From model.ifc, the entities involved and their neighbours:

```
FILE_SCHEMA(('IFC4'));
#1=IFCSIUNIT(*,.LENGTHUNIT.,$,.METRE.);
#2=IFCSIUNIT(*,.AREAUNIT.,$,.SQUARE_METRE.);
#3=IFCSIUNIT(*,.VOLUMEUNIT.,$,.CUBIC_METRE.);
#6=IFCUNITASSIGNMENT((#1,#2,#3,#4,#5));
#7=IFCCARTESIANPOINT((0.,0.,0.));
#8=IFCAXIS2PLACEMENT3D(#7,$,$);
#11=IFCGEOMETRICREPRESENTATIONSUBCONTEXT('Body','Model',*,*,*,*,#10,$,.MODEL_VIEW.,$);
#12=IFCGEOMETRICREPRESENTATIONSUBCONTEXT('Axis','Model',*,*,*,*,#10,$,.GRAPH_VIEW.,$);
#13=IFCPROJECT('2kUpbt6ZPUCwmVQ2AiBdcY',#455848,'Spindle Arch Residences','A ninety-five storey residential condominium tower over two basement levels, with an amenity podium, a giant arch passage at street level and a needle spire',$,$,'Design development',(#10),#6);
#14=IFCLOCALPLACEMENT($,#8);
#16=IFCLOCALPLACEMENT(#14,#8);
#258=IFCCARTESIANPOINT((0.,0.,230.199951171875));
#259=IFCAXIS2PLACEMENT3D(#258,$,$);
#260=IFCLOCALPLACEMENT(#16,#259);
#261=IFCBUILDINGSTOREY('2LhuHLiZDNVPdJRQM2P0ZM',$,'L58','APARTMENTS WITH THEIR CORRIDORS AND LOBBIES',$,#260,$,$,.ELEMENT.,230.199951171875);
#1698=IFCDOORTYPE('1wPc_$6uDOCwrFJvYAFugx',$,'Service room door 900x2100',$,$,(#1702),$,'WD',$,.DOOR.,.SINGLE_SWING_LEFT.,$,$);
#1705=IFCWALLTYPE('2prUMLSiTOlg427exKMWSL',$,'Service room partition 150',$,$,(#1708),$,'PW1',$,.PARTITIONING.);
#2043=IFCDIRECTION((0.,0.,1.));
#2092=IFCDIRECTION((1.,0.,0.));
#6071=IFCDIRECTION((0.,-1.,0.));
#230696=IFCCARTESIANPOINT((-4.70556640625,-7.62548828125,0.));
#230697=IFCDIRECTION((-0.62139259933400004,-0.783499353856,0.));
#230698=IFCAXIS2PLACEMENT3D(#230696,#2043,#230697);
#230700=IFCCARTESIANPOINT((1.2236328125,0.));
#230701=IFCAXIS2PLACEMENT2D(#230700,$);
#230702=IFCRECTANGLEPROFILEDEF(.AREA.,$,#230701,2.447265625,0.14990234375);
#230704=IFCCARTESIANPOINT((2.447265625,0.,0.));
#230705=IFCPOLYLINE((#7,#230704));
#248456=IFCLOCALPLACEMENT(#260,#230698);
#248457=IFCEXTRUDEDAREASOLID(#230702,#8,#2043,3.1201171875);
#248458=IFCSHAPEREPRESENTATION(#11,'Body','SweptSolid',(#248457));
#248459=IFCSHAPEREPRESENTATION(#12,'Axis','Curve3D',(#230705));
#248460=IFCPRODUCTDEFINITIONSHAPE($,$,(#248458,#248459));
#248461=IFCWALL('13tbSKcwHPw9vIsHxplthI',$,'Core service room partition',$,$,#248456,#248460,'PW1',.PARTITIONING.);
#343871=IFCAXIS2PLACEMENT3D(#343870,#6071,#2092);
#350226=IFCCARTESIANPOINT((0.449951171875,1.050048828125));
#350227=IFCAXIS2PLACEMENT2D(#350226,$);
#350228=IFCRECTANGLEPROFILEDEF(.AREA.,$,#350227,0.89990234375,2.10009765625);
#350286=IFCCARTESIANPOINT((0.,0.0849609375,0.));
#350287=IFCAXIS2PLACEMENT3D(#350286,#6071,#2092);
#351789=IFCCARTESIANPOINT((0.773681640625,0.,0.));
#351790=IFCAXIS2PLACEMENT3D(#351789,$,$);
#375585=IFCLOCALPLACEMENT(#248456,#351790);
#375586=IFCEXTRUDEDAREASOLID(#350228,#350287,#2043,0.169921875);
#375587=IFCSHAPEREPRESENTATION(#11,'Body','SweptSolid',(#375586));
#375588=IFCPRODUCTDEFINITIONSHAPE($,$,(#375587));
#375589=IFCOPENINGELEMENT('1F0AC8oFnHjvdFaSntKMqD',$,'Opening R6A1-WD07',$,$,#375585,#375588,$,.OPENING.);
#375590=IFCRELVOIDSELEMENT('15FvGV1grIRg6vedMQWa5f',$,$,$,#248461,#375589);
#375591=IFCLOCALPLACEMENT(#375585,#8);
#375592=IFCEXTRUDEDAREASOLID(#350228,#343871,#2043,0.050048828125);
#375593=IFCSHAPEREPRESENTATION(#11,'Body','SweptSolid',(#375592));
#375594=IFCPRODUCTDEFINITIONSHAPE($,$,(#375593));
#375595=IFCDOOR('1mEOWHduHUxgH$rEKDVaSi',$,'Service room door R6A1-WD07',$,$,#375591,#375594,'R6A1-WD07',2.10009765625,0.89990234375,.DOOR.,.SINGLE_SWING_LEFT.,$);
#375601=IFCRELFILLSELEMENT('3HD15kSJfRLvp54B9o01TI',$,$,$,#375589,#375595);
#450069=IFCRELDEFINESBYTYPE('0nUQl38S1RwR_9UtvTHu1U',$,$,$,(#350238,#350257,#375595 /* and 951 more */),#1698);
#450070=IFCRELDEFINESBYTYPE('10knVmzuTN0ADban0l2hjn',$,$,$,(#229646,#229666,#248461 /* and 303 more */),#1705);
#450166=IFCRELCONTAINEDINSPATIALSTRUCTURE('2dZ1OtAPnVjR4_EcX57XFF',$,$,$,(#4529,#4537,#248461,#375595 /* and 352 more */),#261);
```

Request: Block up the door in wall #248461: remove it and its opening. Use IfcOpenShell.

```python
import ifcopenshell
import ifcopenshell.api.feature
import ifcopenshell.api.root
import ifcopenshell.geom
import ifcopenshell.util.shape

model = ifcopenshell.open("model.ifc")
settings = ifcopenshell.geom.settings()


def volume(element):
    """Net volume in cubic metres, openings subtracted."""
    shape = ifcopenshell.geom.create_shape(settings, element)
    return ifcopenshell.util.shape.get_volume(shape.geometry)


door = model.by_guid("1mEOWHduHUxgH$rEKDVaSi")
opening = door.FillsVoids[0].RelatingOpeningElement
wall = opening.VoidsElements[0].RelatingBuildingElement
before = volume(wall)

ifcopenshell.api.root.remove_product(model, product=door)
ifcopenshell.api.feature.remove_feature(model, feature=opening)

after = volume(wall)

print(f"wall volume {before:.3f} -> {after:.3f} m3")

model.write("model_v2.ifc")
```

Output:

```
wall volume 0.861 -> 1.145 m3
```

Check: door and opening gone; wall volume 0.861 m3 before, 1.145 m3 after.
